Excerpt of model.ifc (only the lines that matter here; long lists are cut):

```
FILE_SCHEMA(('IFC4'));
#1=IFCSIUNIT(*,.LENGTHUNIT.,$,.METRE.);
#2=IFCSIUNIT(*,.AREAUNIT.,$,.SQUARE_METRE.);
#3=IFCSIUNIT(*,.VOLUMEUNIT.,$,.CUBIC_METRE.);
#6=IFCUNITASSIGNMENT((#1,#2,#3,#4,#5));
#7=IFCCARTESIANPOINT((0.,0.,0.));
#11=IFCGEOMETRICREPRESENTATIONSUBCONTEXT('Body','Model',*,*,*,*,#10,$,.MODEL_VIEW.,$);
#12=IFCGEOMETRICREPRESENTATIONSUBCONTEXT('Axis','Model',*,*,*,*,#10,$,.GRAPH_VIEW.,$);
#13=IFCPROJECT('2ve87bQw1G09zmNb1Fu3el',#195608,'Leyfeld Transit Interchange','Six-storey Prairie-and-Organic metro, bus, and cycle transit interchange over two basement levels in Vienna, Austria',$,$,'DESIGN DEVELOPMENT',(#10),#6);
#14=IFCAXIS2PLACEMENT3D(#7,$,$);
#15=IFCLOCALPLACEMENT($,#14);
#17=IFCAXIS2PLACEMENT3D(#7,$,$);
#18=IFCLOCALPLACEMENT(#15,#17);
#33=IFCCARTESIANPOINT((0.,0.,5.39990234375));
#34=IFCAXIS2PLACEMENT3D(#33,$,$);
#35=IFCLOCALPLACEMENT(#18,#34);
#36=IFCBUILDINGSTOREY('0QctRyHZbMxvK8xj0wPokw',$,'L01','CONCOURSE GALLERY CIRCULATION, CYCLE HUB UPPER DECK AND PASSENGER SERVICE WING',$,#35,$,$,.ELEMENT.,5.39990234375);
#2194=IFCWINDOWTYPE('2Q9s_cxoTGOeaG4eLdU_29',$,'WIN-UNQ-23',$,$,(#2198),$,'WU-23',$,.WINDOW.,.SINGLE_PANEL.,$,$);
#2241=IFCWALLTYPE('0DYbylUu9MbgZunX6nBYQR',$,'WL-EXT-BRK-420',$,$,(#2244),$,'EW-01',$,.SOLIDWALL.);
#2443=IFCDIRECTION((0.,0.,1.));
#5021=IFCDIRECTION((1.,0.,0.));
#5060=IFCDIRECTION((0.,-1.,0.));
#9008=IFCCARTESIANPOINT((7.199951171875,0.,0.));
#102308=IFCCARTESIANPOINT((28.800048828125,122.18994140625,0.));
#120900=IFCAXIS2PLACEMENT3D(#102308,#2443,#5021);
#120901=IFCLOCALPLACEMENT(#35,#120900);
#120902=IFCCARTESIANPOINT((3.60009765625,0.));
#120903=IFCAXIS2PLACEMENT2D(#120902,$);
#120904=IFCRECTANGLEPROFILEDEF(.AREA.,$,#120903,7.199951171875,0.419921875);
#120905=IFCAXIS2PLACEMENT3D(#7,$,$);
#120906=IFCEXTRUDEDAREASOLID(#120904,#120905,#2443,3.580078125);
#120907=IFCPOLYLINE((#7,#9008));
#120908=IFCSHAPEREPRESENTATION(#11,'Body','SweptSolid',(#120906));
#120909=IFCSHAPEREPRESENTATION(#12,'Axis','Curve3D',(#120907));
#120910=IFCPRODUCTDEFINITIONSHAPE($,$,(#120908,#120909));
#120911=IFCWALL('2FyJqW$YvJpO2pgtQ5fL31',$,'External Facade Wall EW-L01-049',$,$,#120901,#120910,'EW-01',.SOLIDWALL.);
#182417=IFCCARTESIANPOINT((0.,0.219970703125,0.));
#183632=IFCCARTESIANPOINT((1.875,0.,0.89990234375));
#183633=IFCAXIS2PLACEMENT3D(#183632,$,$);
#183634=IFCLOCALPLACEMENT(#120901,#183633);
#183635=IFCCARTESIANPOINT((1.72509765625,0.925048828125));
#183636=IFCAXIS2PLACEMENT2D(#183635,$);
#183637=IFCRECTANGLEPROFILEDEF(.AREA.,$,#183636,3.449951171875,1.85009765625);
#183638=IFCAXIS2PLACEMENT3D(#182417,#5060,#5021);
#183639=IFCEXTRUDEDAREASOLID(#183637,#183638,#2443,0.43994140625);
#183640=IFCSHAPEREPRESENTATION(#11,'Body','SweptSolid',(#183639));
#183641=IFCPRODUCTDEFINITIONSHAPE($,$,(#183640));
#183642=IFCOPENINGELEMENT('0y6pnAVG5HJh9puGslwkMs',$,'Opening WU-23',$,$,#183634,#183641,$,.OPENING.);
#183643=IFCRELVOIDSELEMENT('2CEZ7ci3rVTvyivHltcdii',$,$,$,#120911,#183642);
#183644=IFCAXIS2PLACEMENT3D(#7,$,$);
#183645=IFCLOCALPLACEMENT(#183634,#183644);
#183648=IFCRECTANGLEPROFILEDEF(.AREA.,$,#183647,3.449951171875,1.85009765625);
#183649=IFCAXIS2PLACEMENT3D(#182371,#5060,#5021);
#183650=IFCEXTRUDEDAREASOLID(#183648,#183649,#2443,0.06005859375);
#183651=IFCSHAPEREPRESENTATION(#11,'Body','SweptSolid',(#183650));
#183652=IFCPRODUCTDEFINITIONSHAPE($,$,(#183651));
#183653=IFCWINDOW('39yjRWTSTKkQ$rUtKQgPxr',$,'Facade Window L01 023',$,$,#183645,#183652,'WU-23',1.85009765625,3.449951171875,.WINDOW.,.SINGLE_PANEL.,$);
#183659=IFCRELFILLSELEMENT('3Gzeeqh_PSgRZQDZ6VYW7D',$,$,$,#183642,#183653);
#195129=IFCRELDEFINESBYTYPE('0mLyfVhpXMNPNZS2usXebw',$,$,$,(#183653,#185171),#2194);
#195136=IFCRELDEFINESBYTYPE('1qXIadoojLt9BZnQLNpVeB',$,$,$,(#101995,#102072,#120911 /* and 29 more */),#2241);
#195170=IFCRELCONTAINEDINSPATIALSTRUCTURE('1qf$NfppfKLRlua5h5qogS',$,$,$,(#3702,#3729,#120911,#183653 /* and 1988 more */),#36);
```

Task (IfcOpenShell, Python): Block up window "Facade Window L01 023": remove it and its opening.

```python
import ifcopenshell
import ifcopenshell.api.feature
import ifcopenshell.api.root
import ifcopenshell.geom
import ifcopenshell.util.shape

model = ifcopenshell.open("model.ifc")
settings = ifcopenshell.geom.settings()


def volume(element):
    """Net volume in cubic metres, openings subtracted."""
    shape = ifcopenshell.geom.create_shape(settings, element)
    return ifcopenshell.util.shape.get_volume(shape.geometry)


window = model.by_guid("39yjRWTSTKkQ$rUtKQgPxr")
opening = window.FillsVoids[0].RelatingOpeningElement
wall = opening.VoidsElements[0].RelatingBuildingElement
before = volume(wall)

ifcopenshell.api.root.remove_product(model, product=window)
ifcopenshell.api.feature.remove_feature(model, feature=opening)

after = volume(wall)

print(f"wall volume {before:.3f} -> {after:.3f} m3")

model.write("model_updated.ifc")
```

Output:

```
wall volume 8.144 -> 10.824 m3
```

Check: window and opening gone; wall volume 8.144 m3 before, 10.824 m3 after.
